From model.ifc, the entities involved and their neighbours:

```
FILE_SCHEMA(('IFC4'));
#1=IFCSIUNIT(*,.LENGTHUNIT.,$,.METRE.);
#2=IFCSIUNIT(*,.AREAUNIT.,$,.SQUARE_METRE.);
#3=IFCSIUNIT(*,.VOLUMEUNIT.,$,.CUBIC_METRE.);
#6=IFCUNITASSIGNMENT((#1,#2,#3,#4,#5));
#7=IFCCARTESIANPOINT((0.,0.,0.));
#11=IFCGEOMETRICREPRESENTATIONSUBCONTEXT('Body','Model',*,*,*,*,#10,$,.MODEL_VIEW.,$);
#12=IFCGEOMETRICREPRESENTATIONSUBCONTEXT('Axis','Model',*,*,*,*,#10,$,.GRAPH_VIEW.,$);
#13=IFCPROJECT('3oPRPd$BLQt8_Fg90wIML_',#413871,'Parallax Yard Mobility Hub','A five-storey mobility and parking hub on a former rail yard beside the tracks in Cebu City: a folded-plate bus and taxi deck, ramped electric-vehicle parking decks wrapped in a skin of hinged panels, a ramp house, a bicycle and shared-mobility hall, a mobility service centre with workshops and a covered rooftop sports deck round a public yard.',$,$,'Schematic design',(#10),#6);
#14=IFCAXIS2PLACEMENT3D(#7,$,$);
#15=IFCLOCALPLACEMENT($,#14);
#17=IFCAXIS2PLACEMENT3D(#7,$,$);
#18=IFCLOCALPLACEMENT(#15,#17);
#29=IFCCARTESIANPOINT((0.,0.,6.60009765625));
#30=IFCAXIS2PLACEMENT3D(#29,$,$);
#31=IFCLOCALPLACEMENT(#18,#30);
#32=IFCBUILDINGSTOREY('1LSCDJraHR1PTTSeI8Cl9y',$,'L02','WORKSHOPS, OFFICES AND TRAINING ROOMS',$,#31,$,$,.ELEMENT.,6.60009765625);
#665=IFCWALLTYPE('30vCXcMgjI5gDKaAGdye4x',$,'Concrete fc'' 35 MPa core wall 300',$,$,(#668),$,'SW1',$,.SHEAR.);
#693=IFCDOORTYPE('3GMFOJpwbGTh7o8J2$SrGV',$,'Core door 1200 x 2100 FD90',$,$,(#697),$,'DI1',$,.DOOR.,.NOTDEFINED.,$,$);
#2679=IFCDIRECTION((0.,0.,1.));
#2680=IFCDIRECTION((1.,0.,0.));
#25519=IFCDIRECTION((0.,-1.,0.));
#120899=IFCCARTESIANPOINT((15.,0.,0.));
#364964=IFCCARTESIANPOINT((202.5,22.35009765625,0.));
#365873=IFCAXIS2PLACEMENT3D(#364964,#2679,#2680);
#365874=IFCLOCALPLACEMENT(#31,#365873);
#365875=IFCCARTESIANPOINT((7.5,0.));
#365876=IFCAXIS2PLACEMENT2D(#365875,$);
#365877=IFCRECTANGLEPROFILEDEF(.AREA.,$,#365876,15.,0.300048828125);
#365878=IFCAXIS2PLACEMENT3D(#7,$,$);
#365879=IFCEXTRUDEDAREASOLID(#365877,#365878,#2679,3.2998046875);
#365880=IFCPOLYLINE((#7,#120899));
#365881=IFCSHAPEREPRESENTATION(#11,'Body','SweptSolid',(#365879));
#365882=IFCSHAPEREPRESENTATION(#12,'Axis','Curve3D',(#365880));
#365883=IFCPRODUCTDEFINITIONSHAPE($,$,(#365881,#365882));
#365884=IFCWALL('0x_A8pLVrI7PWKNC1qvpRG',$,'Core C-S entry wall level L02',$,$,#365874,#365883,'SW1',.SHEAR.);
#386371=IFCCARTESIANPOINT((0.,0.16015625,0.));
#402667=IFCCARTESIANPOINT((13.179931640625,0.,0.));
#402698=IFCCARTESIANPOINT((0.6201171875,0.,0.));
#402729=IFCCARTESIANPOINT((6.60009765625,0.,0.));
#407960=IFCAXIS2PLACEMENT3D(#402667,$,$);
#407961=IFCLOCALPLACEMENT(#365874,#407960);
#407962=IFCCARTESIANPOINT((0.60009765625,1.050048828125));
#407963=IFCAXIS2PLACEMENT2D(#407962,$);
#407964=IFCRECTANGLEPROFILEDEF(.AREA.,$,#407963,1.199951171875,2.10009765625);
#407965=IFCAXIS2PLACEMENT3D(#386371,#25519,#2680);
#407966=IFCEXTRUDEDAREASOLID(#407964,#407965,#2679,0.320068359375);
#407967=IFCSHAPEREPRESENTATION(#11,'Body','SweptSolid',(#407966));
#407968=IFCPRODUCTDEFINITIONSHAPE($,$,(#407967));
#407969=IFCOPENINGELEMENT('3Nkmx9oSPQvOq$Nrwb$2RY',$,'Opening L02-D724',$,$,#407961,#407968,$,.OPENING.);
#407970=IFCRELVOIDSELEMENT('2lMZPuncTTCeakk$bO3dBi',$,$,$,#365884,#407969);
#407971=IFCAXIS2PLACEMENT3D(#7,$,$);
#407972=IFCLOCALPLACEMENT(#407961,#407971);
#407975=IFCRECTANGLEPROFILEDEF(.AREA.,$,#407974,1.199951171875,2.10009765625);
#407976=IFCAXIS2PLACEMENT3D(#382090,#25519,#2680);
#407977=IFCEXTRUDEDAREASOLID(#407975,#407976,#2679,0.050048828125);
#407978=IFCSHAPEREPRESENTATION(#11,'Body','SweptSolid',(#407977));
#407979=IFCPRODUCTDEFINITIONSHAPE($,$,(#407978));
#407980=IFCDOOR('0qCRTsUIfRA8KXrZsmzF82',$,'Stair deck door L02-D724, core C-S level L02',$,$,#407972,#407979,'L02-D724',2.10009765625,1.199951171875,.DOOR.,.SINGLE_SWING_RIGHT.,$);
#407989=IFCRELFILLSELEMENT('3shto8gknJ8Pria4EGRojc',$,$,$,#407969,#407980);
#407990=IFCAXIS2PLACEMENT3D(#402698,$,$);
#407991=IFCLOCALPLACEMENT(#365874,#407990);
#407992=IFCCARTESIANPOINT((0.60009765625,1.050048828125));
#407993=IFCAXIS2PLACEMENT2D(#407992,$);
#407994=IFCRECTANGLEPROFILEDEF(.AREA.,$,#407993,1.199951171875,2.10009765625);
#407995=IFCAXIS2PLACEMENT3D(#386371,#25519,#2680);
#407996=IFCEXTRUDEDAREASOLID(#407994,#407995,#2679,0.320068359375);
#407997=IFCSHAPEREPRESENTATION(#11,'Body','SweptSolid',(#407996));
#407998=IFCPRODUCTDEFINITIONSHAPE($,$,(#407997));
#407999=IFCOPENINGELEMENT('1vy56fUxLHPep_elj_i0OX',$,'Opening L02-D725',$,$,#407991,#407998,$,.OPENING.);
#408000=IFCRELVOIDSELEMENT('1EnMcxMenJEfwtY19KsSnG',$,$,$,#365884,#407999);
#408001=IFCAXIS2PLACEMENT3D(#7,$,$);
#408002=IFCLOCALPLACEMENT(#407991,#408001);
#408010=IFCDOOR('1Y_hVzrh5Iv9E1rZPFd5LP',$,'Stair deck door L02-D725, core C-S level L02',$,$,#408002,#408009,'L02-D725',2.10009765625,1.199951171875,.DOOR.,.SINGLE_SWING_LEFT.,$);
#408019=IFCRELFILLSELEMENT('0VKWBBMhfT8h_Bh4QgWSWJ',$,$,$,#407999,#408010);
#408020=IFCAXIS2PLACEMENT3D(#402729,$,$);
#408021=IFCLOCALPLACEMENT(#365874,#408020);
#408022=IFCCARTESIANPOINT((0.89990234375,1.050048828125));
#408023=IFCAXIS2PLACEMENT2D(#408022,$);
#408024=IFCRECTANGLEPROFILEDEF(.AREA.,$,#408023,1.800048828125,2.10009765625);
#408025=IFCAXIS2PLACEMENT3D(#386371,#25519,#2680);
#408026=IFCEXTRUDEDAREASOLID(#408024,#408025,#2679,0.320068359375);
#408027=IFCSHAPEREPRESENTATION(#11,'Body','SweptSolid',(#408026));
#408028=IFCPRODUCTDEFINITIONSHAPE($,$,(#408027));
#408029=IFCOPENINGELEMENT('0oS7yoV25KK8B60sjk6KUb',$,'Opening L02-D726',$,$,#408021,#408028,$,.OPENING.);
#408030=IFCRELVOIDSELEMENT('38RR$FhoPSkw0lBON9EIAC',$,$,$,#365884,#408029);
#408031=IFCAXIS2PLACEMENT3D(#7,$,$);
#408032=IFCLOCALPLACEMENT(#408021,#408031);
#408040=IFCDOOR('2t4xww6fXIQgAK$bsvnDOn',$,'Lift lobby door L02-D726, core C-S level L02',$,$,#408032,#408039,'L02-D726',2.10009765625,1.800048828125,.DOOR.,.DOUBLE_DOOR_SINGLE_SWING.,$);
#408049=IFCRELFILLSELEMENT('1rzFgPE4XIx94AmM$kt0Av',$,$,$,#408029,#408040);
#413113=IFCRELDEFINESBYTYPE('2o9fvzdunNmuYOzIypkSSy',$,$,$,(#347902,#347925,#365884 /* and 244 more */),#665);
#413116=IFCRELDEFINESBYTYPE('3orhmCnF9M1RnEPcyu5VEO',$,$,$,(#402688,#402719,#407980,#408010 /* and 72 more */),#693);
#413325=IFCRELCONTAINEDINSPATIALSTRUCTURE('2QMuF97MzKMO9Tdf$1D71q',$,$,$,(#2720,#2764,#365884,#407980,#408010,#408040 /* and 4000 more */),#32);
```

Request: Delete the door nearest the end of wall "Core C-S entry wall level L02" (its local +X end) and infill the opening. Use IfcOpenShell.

```python
import ifcopenshell
import ifcopenshell.api.feature
import ifcopenshell.api.root
import ifcopenshell.geom
import ifcopenshell.util.shape

model = ifcopenshell.open("model.ifc")
settings = ifcopenshell.geom.settings()


def volume(element):
    """Net volume in cubic metres, openings subtracted."""
    shape = ifcopenshell.geom.create_shape(settings, element)
    return ifcopenshell.util.shape.get_volume(shape.geometry)


door = model.by_guid("0qCRTsUIfRA8KXrZsmzF82")
opening = door.FillsVoids[0].RelatingOpeningElement
wall = opening.VoidsElements[0].RelatingBuildingElement
before = volume(wall)

ifcopenshell.api.root.remove_product(model, product=door)
ifcopenshell.api.feature.remove_feature(model, feature=opening)

after = volume(wall)

print(f"wall volume {before:.3f} -> {after:.3f} m3")

model.write("model_v2.ifc")
```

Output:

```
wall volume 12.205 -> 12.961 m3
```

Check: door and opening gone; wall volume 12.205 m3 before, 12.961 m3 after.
